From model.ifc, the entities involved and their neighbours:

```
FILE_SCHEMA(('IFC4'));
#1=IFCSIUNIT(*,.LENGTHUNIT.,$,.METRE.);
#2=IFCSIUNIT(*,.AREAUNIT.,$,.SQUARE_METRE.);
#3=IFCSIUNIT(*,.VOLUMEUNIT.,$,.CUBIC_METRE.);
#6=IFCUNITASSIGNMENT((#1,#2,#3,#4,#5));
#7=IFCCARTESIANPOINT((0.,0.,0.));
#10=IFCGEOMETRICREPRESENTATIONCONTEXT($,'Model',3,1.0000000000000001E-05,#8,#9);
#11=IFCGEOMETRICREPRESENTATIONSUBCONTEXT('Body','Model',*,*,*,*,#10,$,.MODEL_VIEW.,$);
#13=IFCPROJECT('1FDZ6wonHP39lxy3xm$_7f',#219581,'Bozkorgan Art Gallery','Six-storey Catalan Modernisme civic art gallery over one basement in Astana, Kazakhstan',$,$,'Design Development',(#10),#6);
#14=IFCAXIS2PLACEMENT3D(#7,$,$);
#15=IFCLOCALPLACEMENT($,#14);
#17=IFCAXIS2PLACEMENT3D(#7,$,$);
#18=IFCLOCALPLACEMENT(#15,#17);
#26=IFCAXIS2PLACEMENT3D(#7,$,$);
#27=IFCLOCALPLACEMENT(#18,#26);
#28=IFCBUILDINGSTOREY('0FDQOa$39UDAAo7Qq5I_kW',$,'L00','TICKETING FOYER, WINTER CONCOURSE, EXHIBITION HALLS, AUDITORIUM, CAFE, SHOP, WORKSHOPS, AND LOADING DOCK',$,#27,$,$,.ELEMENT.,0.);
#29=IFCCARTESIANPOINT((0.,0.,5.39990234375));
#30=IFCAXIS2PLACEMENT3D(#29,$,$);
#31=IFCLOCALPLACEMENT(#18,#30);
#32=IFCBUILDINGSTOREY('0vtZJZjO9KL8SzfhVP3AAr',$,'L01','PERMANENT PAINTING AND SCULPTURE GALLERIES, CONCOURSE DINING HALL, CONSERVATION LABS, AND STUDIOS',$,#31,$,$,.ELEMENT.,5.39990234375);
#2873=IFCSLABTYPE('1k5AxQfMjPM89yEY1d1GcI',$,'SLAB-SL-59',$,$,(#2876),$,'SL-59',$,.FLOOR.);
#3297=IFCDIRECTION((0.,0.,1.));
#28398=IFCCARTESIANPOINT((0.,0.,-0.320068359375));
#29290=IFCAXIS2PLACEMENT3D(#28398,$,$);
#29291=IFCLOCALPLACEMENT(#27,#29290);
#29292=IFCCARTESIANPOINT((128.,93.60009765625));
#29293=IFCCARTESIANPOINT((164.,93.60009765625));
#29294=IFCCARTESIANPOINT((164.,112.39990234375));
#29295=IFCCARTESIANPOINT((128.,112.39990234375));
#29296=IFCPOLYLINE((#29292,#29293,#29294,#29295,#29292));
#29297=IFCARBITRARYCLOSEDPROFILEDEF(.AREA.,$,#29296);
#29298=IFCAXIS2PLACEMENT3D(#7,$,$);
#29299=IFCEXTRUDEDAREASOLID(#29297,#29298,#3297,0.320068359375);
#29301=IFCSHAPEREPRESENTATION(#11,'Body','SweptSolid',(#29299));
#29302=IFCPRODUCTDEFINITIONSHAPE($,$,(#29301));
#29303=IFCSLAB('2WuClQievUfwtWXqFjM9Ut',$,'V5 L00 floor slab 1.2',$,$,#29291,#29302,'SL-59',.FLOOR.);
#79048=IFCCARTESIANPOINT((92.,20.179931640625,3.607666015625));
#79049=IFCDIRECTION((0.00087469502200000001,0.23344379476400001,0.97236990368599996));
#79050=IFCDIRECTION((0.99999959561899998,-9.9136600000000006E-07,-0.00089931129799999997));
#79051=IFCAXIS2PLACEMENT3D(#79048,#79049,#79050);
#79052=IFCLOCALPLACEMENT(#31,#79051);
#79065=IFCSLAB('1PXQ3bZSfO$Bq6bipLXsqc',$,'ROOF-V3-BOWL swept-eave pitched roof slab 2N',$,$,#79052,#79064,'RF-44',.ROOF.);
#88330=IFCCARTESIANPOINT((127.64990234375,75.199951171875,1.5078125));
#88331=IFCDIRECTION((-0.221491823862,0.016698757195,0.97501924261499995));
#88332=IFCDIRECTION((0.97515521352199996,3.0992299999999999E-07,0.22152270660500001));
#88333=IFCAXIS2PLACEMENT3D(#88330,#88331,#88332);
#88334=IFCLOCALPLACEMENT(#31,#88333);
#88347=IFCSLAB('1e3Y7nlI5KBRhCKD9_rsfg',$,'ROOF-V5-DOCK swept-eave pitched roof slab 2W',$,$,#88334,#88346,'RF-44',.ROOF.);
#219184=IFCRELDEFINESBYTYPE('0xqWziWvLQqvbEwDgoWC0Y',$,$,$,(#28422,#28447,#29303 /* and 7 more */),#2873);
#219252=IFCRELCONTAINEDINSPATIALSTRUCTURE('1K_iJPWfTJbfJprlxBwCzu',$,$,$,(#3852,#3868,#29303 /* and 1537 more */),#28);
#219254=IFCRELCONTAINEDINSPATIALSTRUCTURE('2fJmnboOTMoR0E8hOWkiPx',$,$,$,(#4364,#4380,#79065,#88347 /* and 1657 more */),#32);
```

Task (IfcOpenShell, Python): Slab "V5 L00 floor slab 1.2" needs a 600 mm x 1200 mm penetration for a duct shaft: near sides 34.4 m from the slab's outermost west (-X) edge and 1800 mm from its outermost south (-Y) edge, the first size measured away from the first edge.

```python
import numpy as np
import ifcopenshell
import ifcopenshell.api.feature
import ifcopenshell.api.geometry
import ifcopenshell.api.root
import ifcopenshell.geom
import ifcopenshell.util.placement
import ifcopenshell.util.representation
import ifcopenshell.util.shape
import ifcopenshell.util.unit

model = ifcopenshell.open("model.ifc")
unit_scale = ifcopenshell.util.unit.calculate_unit_scale(model)
settings = ifcopenshell.geom.settings()


def volume(element):
    """Net volume in cubic metres, openings subtracted."""
    shape = ifcopenshell.geom.create_shape(settings, element)
    return ifcopenshell.util.shape.get_volume(shape.geometry)


slab = model.by_id(29303)
before = volume(slab)

# Extent in the slab's own axes, in metres. The edges named are its -X and -Y sides.
slab_shape = ifcopenshell.geom.create_shape(settings, slab)
vertices = ifcopenshell.util.shape.get_vertices(slab_shape.geometry)
x_min, y_min, bottom = vertices.min(axis=0)
top = vertices[:, 2].max()

opening = ifcopenshell.api.root.create_entity(model, ifc_class="IfcOpeningElement", name="Duct shaft opening", predefined_type="OPENING")
context = ifcopenshell.util.representation.get_context(model, "Model", "Body", "MODEL_VIEW")
width, depth = 0.6, 1.2
outline = [(0.0, 0.0), (width, 0.0), (width, depth), (0.0, depth), (0.0, 0.0)]
# Overshoot both faces by 50 mm so the cut is clean.
shape = ifcopenshell.api.geometry.add_slab_representation(
    model, context=context, depth=top - bottom + 0.1, polyline=outline
)
ifcopenshell.api.geometry.assign_representation(model, product=opening, representation=shape)

matrix = ifcopenshell.util.placement.get_local_placement(slab.ObjectPlacement)
matrix[:, 3] = matrix @ np.append(np.array([x_min + 34.4, y_min + 1.8, bottom - 0.05]) / unit_scale, 1.0)
ifcopenshell.api.geometry.edit_object_placement(model, product=opening, matrix=matrix, is_si=False)
ifcopenshell.api.feature.add_feature(model, feature=opening, element=slab)

after = volume(slab)

print(f"slab volume {before:.3f} -> {after:.3f} m3")

model.write("model-out.ifc")
```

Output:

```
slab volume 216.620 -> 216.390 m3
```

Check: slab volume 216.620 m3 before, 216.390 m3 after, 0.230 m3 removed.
